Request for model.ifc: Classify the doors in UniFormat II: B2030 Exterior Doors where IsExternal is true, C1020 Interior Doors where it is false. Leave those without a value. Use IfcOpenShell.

First a look at what the model holds.

```python
import ifcopenshell
import ifcopenshell.util.element

model = ifcopenshell.open("model.ifc")
print(model.schema)
print("classifications:", [c.Name for c in model.by_type("IfcClassification")])
values = [ifcopenshell.util.element.get_pset(e, "Pset_DoorCommon", "IsExternal") for e in model.by_type("IfcDoor")]
for value in (True, False, None):
    print("IsExternal", value, values.count(value))
```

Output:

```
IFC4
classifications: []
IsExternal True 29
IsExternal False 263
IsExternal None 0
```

```python
import ifcopenshell
import ifcopenshell.api.classification
import ifcopenshell.util.element

model = ifcopenshell.open("model.ifc")

system = ifcopenshell.api.classification.add_classification(model, classification="UniFormat II")

doors = model.by_type("IfcDoor")
external = {e: ifcopenshell.util.element.get_pset(e, "Pset_DoorCommon", "IsExternal") for e in doors}
for flag, code, name in ((True, "B2030", "Exterior Doors"), (False, "C1020", "Interior Doors")):
    products = [e for e in doors if external[e] is flag]
    ifcopenshell.api.classification.add_reference(
        model, products=products, classification=system, identification=code, name=name
    )
    print(code, len(products))

model.write("model-out.ifc")
```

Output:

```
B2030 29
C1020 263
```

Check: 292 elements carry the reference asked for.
